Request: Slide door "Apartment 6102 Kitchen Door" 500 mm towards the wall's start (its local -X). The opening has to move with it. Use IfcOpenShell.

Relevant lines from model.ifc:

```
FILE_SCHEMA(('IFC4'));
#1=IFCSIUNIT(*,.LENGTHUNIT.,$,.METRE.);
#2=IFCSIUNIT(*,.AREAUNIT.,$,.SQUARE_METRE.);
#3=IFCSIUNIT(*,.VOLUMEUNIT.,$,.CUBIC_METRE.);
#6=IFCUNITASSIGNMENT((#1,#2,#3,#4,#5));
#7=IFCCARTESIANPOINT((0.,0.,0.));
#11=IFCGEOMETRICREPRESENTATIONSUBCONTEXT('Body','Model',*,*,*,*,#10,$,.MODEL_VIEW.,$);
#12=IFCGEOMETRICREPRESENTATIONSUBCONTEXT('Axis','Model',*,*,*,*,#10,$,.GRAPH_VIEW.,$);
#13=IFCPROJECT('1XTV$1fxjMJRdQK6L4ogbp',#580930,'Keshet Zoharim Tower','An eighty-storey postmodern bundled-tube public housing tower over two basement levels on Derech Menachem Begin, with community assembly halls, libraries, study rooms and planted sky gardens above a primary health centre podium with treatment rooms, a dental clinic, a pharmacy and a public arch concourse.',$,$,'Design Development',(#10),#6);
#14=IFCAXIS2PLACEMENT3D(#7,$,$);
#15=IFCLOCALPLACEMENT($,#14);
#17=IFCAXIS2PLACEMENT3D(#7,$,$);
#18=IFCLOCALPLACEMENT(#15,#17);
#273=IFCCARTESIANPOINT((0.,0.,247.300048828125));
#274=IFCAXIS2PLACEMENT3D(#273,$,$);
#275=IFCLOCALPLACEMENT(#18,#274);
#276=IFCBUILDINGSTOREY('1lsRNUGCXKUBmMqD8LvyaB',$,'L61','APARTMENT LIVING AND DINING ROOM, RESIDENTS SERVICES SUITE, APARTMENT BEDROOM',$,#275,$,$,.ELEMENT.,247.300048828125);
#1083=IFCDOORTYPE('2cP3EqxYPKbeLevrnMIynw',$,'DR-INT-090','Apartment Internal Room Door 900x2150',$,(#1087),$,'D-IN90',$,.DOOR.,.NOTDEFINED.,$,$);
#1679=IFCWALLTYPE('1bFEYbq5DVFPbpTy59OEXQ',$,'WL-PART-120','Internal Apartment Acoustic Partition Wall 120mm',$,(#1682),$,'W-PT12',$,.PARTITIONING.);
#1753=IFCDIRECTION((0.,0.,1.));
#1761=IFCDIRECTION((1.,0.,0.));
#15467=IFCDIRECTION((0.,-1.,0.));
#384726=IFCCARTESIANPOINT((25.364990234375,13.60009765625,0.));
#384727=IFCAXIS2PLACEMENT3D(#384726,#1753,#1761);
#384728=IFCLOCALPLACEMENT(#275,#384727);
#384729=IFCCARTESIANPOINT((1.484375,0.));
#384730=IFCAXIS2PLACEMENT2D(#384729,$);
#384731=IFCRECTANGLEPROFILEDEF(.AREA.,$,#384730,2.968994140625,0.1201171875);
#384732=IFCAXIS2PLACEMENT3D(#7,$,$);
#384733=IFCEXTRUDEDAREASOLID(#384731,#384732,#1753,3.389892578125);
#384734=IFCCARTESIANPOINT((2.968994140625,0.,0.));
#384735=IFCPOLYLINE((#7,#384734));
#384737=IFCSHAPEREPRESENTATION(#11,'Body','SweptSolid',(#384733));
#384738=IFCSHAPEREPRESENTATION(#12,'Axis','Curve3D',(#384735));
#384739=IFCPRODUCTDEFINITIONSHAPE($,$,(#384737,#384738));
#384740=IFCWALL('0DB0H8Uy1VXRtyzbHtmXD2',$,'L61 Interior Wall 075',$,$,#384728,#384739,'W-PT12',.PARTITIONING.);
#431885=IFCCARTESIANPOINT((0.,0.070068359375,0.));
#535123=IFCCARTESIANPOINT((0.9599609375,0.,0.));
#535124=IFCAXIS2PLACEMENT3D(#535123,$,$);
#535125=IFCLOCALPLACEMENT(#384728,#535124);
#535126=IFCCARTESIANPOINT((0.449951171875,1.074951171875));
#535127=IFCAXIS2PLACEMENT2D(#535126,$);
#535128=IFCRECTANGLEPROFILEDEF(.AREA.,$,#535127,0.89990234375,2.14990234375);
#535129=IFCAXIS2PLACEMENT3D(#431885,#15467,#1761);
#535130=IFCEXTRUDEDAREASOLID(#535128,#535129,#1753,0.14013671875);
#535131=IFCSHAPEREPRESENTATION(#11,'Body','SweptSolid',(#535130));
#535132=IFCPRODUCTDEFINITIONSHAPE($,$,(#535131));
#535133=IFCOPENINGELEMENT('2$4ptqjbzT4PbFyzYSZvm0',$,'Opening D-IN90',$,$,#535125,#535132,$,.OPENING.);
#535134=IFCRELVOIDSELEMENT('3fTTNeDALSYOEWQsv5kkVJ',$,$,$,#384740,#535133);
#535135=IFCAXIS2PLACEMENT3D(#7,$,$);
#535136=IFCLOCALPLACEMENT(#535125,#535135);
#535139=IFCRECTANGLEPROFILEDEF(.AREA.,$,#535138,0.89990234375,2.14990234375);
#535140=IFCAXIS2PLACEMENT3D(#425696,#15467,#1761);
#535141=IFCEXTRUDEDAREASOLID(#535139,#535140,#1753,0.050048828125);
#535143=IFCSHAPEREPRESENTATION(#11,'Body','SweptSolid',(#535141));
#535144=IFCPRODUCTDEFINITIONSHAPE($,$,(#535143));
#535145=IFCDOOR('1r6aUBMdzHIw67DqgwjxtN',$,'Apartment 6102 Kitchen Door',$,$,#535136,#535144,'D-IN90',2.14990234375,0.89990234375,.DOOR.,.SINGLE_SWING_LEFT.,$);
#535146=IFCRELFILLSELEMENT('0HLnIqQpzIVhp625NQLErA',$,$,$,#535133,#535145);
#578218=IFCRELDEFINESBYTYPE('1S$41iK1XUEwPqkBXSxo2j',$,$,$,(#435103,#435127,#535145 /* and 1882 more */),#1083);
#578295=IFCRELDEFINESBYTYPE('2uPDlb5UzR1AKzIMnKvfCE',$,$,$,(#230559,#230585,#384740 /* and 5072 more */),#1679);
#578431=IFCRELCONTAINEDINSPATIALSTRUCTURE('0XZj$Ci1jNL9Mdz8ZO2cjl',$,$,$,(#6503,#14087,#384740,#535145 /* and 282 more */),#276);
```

```python
import ifcopenshell
import ifcopenshell.api.geometry
import ifcopenshell.util.placement

model = ifcopenshell.open("model.ifc")

door = model.by_guid("1r6aUBMdzHIw67DqgwjxtN")
opening = door.FillsVoids[0].RelatingOpeningElement
wall = opening.VoidsElements[0].RelatingBuildingElement

wall_matrix = ifcopenshell.util.placement.get_local_placement(wall.ObjectPlacement)
shift = wall_matrix[:3, 0] * -0.5
before = ifcopenshell.util.placement.get_local_placement(door.ObjectPlacement)[:3, 3].copy()

# The door is placed relative to its opening, so it follows when the opening moves.
matrix = ifcopenshell.util.placement.get_local_placement(opening.ObjectPlacement)
matrix[:3, 3] += shift
ifcopenshell.api.geometry.edit_object_placement(
    model, product=opening, matrix=matrix, is_si=False, should_transform_children=True
)

after = ifcopenshell.util.placement.get_local_placement(door.ObjectPlacement)[:3, 3]
print("door moved by", (after - before).round(3) + 0.0)

model.write("model_edited.ifc")
```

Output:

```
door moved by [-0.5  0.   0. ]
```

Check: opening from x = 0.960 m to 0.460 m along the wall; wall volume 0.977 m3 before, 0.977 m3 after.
